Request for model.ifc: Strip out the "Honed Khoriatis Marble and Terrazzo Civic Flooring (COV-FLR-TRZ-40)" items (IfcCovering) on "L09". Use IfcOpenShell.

First a look at what the model holds.

```python
import ifcopenshell
import ifcopenshell.util.element

model = ifcopenshell.open("model.ifc")
print(model.schema)
storey = next(s for s in model.by_type("IfcBuildingStorey") if s.Name == "L09")
coverings = [e for e in ifcopenshell.util.element.get_decomposition(storey) if e.is_a("IfcCovering")]
seen = {}
for e in coverings:
    element_type = ifcopenshell.util.element.get_type(e)
    name = element_type.Name if element_type not in (None, e) else None
    seen[name] = seen.get(name, 0) + 1
for name, count in sorted(seen.items(), key=str):
    print(count, "x", name)
```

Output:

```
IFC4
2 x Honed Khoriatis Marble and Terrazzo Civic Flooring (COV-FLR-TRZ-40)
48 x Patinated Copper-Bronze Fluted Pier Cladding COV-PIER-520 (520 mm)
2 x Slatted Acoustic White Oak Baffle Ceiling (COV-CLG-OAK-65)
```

```python
import ifcopenshell
import ifcopenshell.api.root
import ifcopenshell.util.element

model = ifcopenshell.open("model.ifc")

storey = next(s for s in model.by_type("IfcBuildingStorey") if s.Name == "L09")
coverings = [e for e in ifcopenshell.util.element.get_decomposition(storey) if e.is_a("IfcCovering")]
targets = [e for e in coverings if (t := ifcopenshell.util.element.get_type(e)) not in (None, e) and t.Name == "Honed Khoriatis Marble and Terrazzo Civic Flooring (COV-FLR-TRZ-40)"]

for e in targets:
    ifcopenshell.api.root.remove_product(model, product=e)
print(len(targets), "removed")

model.write("model_v2.ifc")
```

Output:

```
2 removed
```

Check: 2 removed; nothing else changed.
